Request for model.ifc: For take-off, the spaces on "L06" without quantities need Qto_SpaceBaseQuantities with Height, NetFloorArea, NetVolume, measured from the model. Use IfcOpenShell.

First a look at what the model holds.

```python
import ifcopenshell
import ifcopenshell.util.element
import ifcopenshell.util.unit

model = ifcopenshell.open("model.ifc")
print(model.schema)
for unit_type in ("LENGTHUNIT", "AREAUNIT", "VOLUMEUNIT"):
    print(unit_type, ifcopenshell.util.unit.calculate_unit_scale(model, unit_type))
storey = next(s for s in model.by_type("IfcBuildingStorey") if s.Name == "L06")
spaces = [e for e in ifcopenshell.util.element.get_decomposition(storey) if e.is_a("IfcSpace")]
for e in sorted(spaces, key=lambda e: e.id()):
    print(e.id(), e.is_a(), e.Name, list(ifcopenshell.util.element.get_psets(e, qtos_only=True)), sep=" | ")
```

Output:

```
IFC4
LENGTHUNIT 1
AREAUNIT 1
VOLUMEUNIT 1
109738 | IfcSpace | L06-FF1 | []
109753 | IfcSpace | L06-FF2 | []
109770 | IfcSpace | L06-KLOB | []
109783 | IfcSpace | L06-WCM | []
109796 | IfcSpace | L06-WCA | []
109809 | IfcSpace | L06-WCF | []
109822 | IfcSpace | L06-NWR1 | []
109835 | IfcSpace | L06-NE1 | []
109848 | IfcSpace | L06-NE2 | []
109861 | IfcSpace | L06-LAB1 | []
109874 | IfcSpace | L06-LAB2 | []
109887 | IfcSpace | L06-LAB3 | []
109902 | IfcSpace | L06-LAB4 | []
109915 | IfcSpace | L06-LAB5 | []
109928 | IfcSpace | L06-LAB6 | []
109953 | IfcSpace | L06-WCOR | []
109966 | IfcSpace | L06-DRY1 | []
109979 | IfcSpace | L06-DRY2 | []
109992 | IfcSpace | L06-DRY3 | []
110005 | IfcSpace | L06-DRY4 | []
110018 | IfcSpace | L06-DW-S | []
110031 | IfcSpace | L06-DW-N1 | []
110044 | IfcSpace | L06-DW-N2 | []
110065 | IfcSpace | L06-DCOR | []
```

```python
import ifcopenshell
import ifcopenshell.api.pset
import ifcopenshell.geom
import ifcopenshell.util.element
import ifcopenshell.util.shape
import ifcopenshell.util.unit

model = ifcopenshell.open("model.ifc")
unit_scale = ifcopenshell.util.unit.calculate_unit_scale(model)
area_scale = ifcopenshell.util.unit.calculate_unit_scale(model, "AREAUNIT")
volume_scale = ifcopenshell.util.unit.calculate_unit_scale(model, "VOLUMEUNIT")
settings = ifcopenshell.geom.settings()

storey = next(s for s in model.by_type("IfcBuildingStorey") if s.Name == "L06")
spaces = [e for e in ifcopenshell.util.element.get_decomposition(storey) if e.is_a("IfcSpace")]

for e in sorted(spaces, key=lambda e: e.id()):
    if ifcopenshell.util.element.get_psets(e, qtos_only=True, should_inherit=False):
        continue
    # Geometry comes back in metres, in the element's own axes.
    shape = ifcopenshell.geom.create_shape(settings, e)
    values = {
        "Height": ifcopenshell.util.shape.get_z(shape.geometry) / unit_scale,
        "NetFloorArea": ifcopenshell.util.shape.get_footprint_area(shape.geometry) / area_scale,
        "NetVolume": ifcopenshell.util.shape.get_volume(shape.geometry) / volume_scale,
    }
    qto = ifcopenshell.api.pset.add_qto(model, product=e, name="Qto_SpaceBaseQuantities")
    ifcopenshell.api.pset.edit_qto(model, qto=qto, properties=values)
    print(e.id(), {k: round(v, 3) for k, v in values.items()})

model.write("model_edited.ifc")
```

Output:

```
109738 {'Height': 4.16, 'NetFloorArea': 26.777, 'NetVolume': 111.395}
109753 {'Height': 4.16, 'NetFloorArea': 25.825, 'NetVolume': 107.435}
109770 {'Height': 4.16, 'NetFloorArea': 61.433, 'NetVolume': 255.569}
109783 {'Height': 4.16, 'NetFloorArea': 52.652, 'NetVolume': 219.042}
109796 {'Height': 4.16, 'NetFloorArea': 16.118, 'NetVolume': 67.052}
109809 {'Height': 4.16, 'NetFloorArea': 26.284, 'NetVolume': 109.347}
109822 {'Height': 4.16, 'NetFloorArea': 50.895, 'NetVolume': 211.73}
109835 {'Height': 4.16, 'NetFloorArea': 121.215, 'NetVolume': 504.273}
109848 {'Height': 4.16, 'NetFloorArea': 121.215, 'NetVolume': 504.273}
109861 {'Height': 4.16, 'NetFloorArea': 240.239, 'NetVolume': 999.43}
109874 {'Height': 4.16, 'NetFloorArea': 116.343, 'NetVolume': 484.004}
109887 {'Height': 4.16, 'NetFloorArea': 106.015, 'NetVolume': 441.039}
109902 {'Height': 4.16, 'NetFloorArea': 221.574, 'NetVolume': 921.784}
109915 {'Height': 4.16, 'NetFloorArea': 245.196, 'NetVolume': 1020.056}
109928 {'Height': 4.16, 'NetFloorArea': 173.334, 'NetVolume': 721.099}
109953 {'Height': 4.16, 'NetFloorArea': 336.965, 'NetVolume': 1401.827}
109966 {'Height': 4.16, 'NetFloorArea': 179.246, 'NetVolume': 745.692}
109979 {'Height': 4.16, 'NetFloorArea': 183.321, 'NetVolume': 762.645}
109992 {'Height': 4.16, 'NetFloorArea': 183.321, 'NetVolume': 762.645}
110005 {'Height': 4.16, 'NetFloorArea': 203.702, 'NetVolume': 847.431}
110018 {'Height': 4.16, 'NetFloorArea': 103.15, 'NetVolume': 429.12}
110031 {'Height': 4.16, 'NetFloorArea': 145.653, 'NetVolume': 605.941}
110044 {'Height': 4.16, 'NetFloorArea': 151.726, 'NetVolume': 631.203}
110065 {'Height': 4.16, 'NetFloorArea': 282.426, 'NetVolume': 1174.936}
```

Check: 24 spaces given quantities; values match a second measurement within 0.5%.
